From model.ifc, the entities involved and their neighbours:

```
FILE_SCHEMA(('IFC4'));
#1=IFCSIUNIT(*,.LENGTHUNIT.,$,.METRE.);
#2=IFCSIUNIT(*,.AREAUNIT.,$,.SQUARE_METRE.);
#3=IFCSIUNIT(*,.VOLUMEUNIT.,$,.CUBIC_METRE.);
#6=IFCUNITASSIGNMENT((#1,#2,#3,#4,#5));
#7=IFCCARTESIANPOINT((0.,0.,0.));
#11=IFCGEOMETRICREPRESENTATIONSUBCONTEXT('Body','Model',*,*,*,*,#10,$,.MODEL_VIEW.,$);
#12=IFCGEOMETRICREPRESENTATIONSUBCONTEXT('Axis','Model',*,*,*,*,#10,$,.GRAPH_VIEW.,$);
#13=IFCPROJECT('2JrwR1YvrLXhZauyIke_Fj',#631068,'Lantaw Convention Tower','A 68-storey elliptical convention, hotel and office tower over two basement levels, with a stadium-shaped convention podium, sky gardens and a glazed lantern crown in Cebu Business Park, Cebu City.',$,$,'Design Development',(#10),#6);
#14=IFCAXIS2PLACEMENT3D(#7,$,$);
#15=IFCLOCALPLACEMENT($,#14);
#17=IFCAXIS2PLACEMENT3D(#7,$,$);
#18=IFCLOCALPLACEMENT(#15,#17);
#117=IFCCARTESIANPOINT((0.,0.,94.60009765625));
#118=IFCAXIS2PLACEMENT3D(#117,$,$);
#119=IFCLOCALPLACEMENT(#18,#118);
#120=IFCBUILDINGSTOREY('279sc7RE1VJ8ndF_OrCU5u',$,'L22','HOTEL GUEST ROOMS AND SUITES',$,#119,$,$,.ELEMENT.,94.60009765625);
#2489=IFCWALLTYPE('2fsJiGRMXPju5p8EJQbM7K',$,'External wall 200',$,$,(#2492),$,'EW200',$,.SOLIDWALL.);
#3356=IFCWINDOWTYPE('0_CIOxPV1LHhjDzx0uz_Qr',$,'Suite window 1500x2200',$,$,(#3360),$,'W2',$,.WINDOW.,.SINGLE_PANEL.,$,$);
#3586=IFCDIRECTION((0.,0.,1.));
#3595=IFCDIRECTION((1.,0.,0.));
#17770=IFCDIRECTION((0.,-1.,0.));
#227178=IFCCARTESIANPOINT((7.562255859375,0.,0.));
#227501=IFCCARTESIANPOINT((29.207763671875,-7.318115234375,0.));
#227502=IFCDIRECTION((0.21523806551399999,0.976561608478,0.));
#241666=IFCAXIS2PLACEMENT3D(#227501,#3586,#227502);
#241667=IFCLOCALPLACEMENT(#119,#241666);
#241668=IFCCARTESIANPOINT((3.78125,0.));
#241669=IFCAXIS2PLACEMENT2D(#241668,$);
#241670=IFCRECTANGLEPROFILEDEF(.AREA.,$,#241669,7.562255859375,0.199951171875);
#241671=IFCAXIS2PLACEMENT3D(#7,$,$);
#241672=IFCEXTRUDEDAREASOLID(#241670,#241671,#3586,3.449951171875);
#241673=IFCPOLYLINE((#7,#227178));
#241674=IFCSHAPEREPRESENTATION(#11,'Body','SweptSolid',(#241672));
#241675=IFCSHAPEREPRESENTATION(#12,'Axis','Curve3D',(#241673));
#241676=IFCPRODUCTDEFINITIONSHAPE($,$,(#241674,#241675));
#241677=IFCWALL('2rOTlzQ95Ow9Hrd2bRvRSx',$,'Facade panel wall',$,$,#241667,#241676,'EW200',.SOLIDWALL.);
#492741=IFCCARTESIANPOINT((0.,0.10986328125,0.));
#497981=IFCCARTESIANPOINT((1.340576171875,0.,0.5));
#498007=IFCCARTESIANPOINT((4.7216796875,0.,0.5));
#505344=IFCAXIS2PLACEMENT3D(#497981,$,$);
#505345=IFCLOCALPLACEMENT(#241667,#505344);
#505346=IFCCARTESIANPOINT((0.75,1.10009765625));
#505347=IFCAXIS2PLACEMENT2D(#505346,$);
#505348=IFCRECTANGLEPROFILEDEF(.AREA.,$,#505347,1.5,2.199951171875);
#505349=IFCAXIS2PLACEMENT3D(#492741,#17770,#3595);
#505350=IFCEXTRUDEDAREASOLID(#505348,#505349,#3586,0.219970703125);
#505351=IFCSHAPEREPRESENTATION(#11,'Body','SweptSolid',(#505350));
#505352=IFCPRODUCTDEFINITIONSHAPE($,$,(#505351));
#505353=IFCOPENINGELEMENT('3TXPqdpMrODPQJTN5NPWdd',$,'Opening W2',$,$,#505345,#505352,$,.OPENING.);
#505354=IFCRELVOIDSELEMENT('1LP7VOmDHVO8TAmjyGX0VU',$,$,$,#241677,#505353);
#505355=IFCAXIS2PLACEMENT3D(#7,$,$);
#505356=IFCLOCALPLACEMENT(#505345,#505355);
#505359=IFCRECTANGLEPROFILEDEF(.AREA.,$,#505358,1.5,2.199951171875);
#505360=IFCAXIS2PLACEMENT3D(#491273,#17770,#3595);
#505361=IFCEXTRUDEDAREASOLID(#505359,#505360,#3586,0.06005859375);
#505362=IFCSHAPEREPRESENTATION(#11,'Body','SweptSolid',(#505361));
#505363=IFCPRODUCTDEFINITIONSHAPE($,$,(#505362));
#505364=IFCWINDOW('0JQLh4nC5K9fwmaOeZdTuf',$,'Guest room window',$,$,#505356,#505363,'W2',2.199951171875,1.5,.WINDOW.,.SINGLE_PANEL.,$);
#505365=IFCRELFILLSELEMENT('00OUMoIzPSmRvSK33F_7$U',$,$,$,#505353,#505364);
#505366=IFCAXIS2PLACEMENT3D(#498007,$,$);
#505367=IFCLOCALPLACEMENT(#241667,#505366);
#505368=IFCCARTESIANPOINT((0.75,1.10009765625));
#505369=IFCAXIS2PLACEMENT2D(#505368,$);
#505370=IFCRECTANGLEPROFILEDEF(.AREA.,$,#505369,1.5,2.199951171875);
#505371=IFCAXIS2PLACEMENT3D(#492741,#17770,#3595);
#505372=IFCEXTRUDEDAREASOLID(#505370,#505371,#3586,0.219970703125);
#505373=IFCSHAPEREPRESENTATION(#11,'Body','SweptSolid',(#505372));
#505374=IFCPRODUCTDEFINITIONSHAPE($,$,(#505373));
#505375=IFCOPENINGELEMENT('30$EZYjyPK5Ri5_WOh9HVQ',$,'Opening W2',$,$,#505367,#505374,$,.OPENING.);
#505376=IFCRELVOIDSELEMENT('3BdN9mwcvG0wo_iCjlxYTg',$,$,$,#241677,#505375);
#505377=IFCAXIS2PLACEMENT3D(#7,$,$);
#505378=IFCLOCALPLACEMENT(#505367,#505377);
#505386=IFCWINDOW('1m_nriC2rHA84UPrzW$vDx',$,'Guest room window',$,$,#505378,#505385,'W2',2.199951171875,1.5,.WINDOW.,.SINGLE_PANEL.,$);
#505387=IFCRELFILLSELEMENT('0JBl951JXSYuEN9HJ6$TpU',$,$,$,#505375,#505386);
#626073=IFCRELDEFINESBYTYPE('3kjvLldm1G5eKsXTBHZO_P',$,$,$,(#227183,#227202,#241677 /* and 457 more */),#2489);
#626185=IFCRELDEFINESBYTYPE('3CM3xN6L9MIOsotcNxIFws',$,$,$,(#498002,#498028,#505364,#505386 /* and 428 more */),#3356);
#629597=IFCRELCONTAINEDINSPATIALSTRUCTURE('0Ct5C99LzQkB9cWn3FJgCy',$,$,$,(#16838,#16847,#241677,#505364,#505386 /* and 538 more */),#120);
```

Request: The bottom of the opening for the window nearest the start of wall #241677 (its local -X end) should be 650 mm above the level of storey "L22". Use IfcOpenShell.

```python
import numpy as np
import ifcopenshell
import ifcopenshell.api.geometry
import ifcopenshell.geom
import ifcopenshell.util.element
import ifcopenshell.util.placement
import ifcopenshell.util.shape
import ifcopenshell.util.unit

model = ifcopenshell.open("model.ifc")
unit_scale = ifcopenshell.util.unit.calculate_unit_scale(model)

window = model.by_id(505364)
opening = window.FillsVoids[0].RelatingOpeningElement
storey = ifcopenshell.util.element.get_container(window, ifc_class="IfcBuildingStorey")
level = ifcopenshell.util.placement.get_local_placement(storey.ObjectPlacement)[2, 3]

# The opening's origin need not be at the sill, so measure its lowest point.
shape = ifcopenshell.geom.create_shape(ifcopenshell.geom.settings(), opening)
bottom = ifcopenshell.util.shape.get_shape_bottom_elevation(shape, shape.geometry) / unit_scale
dz = level + 0.65 / unit_scale - bottom

shift = np.array([0.0, 0.0, dz])
# The window is placed relative to its opening, so it follows when the opening moves.
matrix = ifcopenshell.util.placement.get_local_placement(opening.ObjectPlacement)
matrix[:3, 3] += shift
ifcopenshell.api.geometry.edit_object_placement(
    model, product=opening, matrix=matrix, is_si=False, should_transform_children=True
)

print(f"moved by {dz * unit_scale:+.3f} m")

model.write("model_v2.ifc")
```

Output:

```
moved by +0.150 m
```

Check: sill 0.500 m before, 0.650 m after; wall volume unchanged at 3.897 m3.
